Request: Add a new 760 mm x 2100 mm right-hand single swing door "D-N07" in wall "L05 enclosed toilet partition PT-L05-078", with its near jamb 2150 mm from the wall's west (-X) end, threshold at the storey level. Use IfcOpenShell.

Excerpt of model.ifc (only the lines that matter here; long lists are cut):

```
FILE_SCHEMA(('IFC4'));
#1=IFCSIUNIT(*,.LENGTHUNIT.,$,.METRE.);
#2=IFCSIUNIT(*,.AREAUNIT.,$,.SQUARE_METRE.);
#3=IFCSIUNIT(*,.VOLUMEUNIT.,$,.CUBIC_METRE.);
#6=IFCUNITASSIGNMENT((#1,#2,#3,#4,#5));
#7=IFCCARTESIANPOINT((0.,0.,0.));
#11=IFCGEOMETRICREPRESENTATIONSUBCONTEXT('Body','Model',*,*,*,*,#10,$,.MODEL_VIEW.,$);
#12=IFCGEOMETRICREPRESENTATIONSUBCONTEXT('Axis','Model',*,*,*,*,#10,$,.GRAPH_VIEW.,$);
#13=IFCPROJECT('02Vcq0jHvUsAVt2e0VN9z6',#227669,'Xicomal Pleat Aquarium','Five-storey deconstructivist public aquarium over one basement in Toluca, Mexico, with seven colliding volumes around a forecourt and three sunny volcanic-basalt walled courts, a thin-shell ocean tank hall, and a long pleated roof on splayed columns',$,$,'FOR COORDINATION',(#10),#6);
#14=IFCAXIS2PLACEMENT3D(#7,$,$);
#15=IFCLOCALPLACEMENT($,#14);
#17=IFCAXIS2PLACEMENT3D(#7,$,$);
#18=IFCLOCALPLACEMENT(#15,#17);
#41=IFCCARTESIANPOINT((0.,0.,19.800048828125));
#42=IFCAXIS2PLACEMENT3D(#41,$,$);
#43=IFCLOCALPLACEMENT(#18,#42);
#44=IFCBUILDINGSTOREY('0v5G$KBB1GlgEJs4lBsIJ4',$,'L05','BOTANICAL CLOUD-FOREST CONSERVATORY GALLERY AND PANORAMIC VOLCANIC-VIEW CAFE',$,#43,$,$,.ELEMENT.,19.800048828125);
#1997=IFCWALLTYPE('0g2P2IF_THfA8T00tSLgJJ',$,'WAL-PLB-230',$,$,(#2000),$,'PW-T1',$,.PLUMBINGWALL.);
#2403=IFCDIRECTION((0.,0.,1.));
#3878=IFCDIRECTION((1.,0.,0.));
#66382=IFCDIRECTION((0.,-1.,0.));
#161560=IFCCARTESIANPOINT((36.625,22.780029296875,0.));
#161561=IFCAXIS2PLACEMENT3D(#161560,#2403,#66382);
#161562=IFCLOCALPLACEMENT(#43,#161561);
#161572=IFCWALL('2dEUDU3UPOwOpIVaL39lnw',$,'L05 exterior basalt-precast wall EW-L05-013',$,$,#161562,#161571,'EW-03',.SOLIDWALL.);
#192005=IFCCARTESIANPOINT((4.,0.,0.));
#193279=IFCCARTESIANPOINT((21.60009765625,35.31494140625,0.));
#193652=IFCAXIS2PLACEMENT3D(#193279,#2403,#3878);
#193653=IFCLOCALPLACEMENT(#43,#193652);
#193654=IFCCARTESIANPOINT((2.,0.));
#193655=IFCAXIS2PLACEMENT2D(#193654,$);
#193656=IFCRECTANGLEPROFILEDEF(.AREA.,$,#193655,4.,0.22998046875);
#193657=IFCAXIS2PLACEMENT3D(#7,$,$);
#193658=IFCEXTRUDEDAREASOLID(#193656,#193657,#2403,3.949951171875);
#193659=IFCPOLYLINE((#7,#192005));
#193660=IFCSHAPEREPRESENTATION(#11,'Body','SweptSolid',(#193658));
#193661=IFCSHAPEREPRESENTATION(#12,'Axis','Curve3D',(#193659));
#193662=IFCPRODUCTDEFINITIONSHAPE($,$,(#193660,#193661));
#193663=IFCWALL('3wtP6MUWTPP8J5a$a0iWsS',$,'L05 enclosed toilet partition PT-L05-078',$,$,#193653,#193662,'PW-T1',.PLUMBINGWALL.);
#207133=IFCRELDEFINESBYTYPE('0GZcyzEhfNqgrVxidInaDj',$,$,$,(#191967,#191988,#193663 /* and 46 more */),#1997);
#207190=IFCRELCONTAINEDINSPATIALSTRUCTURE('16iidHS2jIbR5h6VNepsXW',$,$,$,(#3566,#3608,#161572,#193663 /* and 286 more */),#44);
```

```python
import numpy as np
import ifcopenshell
import ifcopenshell.api.feature
import ifcopenshell.api.geometry
import ifcopenshell.api.root
import ifcopenshell.api.spatial
import ifcopenshell.geom
import ifcopenshell.util.element
import ifcopenshell.util.placement
import ifcopenshell.util.representation
import ifcopenshell.util.shape
import ifcopenshell.util.unit

model = ifcopenshell.open("model.ifc")
unit_scale = ifcopenshell.util.unit.calculate_unit_scale(model)
settings = ifcopenshell.geom.settings()


def volume(element):
    """Net volume in cubic metres, openings subtracted."""
    shape = ifcopenshell.geom.create_shape(settings, element)
    return ifcopenshell.util.shape.get_volume(shape.geometry)


wall = model.by_guid("3wtP6MUWTPP8J5a$a0iWsS")
storey = ifcopenshell.util.element.get_container(wall, ifc_class="IfcBuildingStorey")
context = ifcopenshell.util.representation.get_context(model, "Model", "Body", "MODEL_VIEW")
before = volume(wall)

width, height, from_end, sill = 0.76, 2.1, 2.15, 0.0  # metres

# The wall runs along its own X axis, and the end named is its -X end.
wall_shape = ifcopenshell.geom.create_shape(settings, wall)
x, y, z = ifcopenshell.util.shape.get_vertices(wall_shape.geometry).T
start = x.min() + from_end
face, thickness = float(y.min()), float(y.max() - y.min())
wall_matrix = ifcopenshell.util.placement.get_local_placement(wall.ObjectPlacement)
level = ifcopenshell.util.placement.get_local_placement(storey.ObjectPlacement)[2, 3]


def in_wall(x, y):
    """Placement at x, y metres in the wall's axes, at sill height."""
    matrix = wall_matrix.copy()
    matrix[:, 3] = wall_matrix @ np.array([x / unit_scale, y / unit_scale, 0.0, 1.0])
    matrix[2, 3] = level + sill / unit_scale
    return matrix


# Opening: a box that overshoots both wall faces by 50 mm.
opening = ifcopenshell.api.root.create_entity(model, ifc_class="IfcOpeningElement", predefined_type="OPENING")
box = ifcopenshell.api.geometry.add_wall_representation(
    model, context=context, length=width, height=height, thickness=thickness + 0.1
)
ifcopenshell.api.geometry.assign_representation(model, product=opening, representation=box)
ifcopenshell.api.geometry.edit_object_placement(model, product=opening, matrix=in_wall(start, face - 0.05), is_si=False)
ifcopenshell.api.feature.add_feature(model, feature=opening, element=wall)

door = ifcopenshell.api.root.create_entity(model, ifc_class="IfcDoor", name="D-N07", predefined_type="DOOR")
door.OverallWidth, door.OverallHeight = width / unit_scale, height / unit_scale
door.OperationType = "SINGLE_SWING_RIGHT"
body = ifcopenshell.api.geometry.add_door_representation(
    model,
    context=context,
    overall_width=door.OverallWidth,
    overall_height=door.OverallHeight,
    operation_type="SINGLE_SWING_RIGHT",
    lining_properties={"LiningDepth": thickness / unit_scale, "ThresholdDepth": thickness / unit_scale},
)
ifcopenshell.api.geometry.assign_representation(model, product=door, representation=body)
ifcopenshell.api.spatial.assign_container(model, products=[door], relating_structure=storey)
ifcopenshell.api.feature.add_filling(model, opening=opening, element=door)

# The lining spans the wall, so the door starts at the wall face.
ifcopenshell.api.geometry.edit_object_placement(model, product=door, matrix=in_wall(start, face), is_si=False)

after = volume(wall)

print(f"wall volume {before:.3f} -> {after:.3f} m3")

model.write("model_updated.ifc")
```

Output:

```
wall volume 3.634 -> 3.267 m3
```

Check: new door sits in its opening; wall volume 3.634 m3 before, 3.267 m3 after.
